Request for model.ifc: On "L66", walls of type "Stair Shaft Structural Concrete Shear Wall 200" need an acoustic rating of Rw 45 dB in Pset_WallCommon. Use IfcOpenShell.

First a look at what the model holds.

```python
import ifcopenshell
import ifcopenshell.util.element

model = ifcopenshell.open("model.ifc")
print(model.schema)
storey = next(s for s in model.by_type("IfcBuildingStorey") if s.Name == "L66")
walls = [e for e in ifcopenshell.util.element.get_decomposition(storey) if e.is_a("IfcWall")]
seen = {}
for e in walls:
    element_type = ifcopenshell.util.element.get_type(e)
    key = (element_type.Name if element_type != e and element_type else None, ifcopenshell.util.element.get_pset(e, "Pset_WallCommon", "AcousticRating"))
    seen[key] = seen.get(key, 0) + 1
for (name, value), count in sorted(seen.items(), key=str):
    print(count, "x", name, "|", value)
```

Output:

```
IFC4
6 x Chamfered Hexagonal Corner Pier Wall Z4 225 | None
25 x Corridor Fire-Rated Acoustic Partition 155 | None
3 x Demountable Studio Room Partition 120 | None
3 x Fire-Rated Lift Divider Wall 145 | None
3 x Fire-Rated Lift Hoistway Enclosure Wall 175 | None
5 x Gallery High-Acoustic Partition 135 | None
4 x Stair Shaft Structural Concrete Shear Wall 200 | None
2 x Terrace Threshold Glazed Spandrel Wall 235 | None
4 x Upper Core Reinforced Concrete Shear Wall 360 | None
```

```python
import ifcopenshell
import ifcopenshell.api.pset
import ifcopenshell.util.element

model = ifcopenshell.open("model.ifc")

storey = next(s for s in model.by_type("IfcBuildingStorey") if s.Name == "L66")
walls = [e for e in ifcopenshell.util.element.get_decomposition(storey) if e.is_a("IfcWall")]

count = 0
for e in walls:
    element_type = ifcopenshell.util.element.get_type(e)
    if element_type in (None, e) or element_type.Name != "Stair Shaft Structural Concrete Shear Wall 200":
        continue
    # add_pset returns the element's existing set when there is one.
    pset = ifcopenshell.api.pset.add_pset(model, product=e, name="Pset_WallCommon")
    ifcopenshell.api.pset.edit_pset(model, pset=pset, properties={"AcousticRating": "Rw 45 dB"})
    count += 1

print(count, "walls updated")

model.write("model_edited.ifc")
```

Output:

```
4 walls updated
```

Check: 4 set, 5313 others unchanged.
